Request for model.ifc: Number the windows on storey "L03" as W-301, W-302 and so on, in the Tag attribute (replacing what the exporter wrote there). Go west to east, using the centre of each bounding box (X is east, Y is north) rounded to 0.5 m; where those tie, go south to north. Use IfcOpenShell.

First a look at what the model holds.

```python
import ifcopenshell
import ifcopenshell.util.element
import ifcopenshell.util.placement

model = ifcopenshell.open("model.ifc")
print(model.schema)
storey = next(s for s in model.by_type("IfcBuildingStorey") if s.Name == "L03")
windows = [e for e in ifcopenshell.util.element.get_decomposition(storey) if e.is_a("IfcWindow")]
for e in sorted(windows, key=lambda e: e.id()):
    origin = ifcopenshell.util.placement.get_local_placement(e.ObjectPlacement)[:3, 3]
    print(e.id(), e.Tag, e.Name, origin.round(2) + 0.0, sep=" | ")
```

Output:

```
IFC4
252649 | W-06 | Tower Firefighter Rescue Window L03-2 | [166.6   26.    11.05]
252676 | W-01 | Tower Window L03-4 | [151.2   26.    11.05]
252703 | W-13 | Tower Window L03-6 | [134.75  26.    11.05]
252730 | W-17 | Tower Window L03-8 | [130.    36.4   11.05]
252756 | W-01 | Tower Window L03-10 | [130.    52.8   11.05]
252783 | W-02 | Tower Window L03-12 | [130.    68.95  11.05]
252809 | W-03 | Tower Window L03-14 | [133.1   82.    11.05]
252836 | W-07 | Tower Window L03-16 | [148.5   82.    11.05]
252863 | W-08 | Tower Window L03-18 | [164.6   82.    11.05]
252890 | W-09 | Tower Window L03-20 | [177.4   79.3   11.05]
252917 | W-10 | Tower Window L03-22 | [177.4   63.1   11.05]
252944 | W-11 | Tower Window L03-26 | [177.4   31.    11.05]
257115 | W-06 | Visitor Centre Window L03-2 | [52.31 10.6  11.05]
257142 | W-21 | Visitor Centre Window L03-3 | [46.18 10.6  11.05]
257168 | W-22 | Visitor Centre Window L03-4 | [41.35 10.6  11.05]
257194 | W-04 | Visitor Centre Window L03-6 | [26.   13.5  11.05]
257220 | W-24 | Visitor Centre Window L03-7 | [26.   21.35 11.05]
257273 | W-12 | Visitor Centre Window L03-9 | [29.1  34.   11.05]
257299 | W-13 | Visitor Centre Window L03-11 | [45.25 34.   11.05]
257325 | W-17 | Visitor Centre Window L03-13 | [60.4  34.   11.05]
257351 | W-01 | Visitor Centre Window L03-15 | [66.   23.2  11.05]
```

```python
import ifcopenshell
import ifcopenshell.geom
import ifcopenshell.util.element
import ifcopenshell.util.shape

model = ifcopenshell.open("model.ifc")
settings = ifcopenshell.geom.settings()
settings.set("use-world-coords", True)


def centre(element):
    shape = ifcopenshell.geom.create_shape(settings, element)
    return ifcopenshell.util.shape.get_bbox_centroid(shape.geometry)


storey = next(s for s in model.by_type("IfcBuildingStorey") if s.Name == "L03")
windows = [e for e in ifcopenshell.util.element.get_decomposition(storey) if e.is_a("IfcWindow")]

# Insertion points can sit at a corner or the storey origin, so sort by the geometry (in metres).
centres = {e: centre(e) for e in windows}
windows.sort(key=lambda e: (round(centres[e][0] / 0.5), centres[e][1]))

for i, e in enumerate(windows, start=1):
    number = f"W-3{i:02d}"
    e.Tag = number
    print(e.id(), number)

model.write("model-out.ifc")
```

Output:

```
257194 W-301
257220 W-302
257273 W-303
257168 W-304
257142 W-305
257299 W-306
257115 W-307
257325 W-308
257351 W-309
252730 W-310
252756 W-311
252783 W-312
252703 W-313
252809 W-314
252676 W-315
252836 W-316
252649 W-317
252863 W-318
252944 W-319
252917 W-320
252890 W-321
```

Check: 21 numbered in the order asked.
